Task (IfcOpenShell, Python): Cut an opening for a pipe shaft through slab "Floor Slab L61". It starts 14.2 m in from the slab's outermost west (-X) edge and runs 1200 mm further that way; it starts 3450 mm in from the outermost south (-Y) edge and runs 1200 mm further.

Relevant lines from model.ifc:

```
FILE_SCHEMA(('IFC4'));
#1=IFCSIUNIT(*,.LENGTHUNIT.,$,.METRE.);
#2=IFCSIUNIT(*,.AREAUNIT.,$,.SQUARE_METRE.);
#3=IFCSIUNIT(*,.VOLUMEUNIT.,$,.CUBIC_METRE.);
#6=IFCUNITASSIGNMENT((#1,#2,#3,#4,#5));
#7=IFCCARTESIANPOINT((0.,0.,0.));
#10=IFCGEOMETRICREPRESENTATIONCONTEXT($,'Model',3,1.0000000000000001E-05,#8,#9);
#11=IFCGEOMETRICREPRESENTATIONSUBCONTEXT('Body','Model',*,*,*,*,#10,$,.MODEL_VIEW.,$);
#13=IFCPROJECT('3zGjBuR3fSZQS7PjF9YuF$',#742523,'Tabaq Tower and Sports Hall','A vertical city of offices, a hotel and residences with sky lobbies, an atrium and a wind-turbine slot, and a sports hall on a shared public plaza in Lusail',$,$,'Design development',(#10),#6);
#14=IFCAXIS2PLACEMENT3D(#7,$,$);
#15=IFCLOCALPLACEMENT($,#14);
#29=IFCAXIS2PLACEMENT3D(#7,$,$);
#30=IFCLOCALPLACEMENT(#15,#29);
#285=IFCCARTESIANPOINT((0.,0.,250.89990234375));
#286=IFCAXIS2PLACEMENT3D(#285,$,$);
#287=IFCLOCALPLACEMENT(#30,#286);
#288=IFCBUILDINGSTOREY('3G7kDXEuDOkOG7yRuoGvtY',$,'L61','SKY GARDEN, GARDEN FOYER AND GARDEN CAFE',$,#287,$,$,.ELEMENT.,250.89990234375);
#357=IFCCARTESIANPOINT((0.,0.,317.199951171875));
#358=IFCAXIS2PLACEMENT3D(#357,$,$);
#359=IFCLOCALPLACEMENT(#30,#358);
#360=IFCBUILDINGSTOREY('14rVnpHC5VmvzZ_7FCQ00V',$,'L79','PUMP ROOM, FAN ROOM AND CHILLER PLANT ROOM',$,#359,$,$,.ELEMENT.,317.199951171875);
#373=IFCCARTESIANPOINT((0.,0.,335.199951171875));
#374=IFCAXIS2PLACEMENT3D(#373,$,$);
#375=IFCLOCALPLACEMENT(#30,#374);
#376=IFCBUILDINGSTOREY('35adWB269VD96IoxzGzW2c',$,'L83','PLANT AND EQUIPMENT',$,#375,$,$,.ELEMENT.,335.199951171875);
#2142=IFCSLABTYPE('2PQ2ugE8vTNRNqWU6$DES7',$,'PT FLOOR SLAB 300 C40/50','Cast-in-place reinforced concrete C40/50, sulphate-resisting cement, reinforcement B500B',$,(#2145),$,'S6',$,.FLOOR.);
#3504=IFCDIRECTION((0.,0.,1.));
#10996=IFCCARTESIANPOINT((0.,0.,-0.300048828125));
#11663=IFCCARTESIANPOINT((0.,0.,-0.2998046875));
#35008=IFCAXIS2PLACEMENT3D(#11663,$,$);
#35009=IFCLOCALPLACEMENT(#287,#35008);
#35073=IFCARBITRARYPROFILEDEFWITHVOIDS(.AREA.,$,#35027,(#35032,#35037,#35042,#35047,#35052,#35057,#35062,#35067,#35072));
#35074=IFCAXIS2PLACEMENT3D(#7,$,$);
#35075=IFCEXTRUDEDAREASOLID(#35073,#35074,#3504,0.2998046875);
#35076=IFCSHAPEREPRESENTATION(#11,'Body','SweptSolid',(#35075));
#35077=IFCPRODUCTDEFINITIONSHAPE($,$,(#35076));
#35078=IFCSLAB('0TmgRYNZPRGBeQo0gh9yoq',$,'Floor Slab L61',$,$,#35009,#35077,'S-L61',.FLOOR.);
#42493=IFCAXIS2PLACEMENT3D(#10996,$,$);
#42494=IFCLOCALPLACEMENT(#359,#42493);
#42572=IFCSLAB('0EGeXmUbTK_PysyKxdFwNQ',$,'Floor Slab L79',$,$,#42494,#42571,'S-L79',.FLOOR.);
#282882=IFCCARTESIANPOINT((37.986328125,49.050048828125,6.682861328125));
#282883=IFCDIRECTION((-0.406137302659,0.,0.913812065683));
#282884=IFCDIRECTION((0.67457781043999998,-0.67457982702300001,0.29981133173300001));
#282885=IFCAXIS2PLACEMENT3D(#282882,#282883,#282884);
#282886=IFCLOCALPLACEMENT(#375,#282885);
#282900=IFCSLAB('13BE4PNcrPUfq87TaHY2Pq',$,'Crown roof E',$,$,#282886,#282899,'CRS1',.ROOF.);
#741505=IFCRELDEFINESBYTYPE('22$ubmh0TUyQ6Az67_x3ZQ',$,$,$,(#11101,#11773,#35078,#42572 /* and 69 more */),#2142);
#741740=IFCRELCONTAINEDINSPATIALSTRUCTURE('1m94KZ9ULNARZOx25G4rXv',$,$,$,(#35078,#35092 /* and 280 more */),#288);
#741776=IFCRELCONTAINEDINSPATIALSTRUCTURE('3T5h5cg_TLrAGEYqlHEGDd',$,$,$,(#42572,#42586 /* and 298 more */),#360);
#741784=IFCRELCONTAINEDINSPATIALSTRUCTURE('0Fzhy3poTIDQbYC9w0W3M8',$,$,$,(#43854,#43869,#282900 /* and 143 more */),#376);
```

```python
import numpy as np
import ifcopenshell
import ifcopenshell.api.feature
import ifcopenshell.api.geometry
import ifcopenshell.api.root
import ifcopenshell.geom
import ifcopenshell.util.placement
import ifcopenshell.util.representation
import ifcopenshell.util.shape
import ifcopenshell.util.unit

model = ifcopenshell.open("model.ifc")
unit_scale = ifcopenshell.util.unit.calculate_unit_scale(model)
settings = ifcopenshell.geom.settings()


def volume(element):
    """Net volume in cubic metres, openings subtracted."""
    shape = ifcopenshell.geom.create_shape(settings, element)
    return ifcopenshell.util.shape.get_volume(shape.geometry)


slab = model.by_id(35078)
before = volume(slab)

# Extent in the slab's own axes, in metres. The edges named are its -X and -Y sides.
slab_shape = ifcopenshell.geom.create_shape(settings, slab)
vertices = ifcopenshell.util.shape.get_vertices(slab_shape.geometry)
x_min, y_min, bottom = vertices.min(axis=0)
top = vertices[:, 2].max()

opening = ifcopenshell.api.root.create_entity(model, ifc_class="IfcOpeningElement", name="Pipe shaft opening", predefined_type="OPENING")
context = ifcopenshell.util.representation.get_context(model, "Model", "Body", "MODEL_VIEW")
width, depth = 1.2, 1.2
outline = [(0.0, 0.0), (width, 0.0), (width, depth), (0.0, depth), (0.0, 0.0)]
# Overshoot both faces by 50 mm so the cut is clean.
shape = ifcopenshell.api.geometry.add_slab_representation(
    model, context=context, depth=top - bottom + 0.1, polyline=outline
)
ifcopenshell.api.geometry.assign_representation(model, product=opening, representation=shape)

matrix = ifcopenshell.util.placement.get_local_placement(slab.ObjectPlacement)
matrix[:, 3] = matrix @ np.append(np.array([x_min + 14.2, y_min + 3.45, bottom - 0.05]) / unit_scale, 1.0)
ifcopenshell.api.geometry.edit_object_placement(model, product=opening, matrix=matrix, is_si=False)
ifcopenshell.api.feature.add_feature(model, feature=opening, element=slab)

after = volume(slab)

print(f"slab volume {before:.3f} -> {after:.3f} m3")

model.write("model-out.ifc")
```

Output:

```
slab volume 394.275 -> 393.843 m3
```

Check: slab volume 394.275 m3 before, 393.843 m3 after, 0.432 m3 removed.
